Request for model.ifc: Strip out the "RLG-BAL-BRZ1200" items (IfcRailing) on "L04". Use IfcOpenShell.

First a look at what the model holds.

```python
import ifcopenshell
import ifcopenshell.util.element

model = ifcopenshell.open("model.ifc")
print(model.schema)
storey = next(s for s in model.by_type("IfcBuildingStorey") if s.Name == "L04")
railings = [e for e in ifcopenshell.util.element.get_decomposition(storey) if e.is_a("IfcRailing")]
seen = {}
for e in railings:
    element_type = ifcopenshell.util.element.get_type(e)
    name = element_type.Name if element_type not in (None, e) else None
    seen[name] = seen.get(name, 0) + 1
for name, count in sorted(seen.items(), key=str):
    print(count, "x", name)
```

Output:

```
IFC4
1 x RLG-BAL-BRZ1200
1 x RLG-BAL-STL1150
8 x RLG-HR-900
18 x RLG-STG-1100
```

```python
import ifcopenshell
import ifcopenshell.api.root
import ifcopenshell.util.element

model = ifcopenshell.open("model.ifc")

storey = next(s for s in model.by_type("IfcBuildingStorey") if s.Name == "L04")
railings = [e for e in ifcopenshell.util.element.get_decomposition(storey) if e.is_a("IfcRailing")]
targets = [e for e in railings if (t := ifcopenshell.util.element.get_type(e)) not in (None, e) and t.Name == "RLG-BAL-BRZ1200"]

for e in targets:
    ifcopenshell.api.root.remove_product(model, product=e)
print(len(targets), "removed")

model.write("model_updated.ifc")
```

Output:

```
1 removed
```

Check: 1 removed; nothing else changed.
